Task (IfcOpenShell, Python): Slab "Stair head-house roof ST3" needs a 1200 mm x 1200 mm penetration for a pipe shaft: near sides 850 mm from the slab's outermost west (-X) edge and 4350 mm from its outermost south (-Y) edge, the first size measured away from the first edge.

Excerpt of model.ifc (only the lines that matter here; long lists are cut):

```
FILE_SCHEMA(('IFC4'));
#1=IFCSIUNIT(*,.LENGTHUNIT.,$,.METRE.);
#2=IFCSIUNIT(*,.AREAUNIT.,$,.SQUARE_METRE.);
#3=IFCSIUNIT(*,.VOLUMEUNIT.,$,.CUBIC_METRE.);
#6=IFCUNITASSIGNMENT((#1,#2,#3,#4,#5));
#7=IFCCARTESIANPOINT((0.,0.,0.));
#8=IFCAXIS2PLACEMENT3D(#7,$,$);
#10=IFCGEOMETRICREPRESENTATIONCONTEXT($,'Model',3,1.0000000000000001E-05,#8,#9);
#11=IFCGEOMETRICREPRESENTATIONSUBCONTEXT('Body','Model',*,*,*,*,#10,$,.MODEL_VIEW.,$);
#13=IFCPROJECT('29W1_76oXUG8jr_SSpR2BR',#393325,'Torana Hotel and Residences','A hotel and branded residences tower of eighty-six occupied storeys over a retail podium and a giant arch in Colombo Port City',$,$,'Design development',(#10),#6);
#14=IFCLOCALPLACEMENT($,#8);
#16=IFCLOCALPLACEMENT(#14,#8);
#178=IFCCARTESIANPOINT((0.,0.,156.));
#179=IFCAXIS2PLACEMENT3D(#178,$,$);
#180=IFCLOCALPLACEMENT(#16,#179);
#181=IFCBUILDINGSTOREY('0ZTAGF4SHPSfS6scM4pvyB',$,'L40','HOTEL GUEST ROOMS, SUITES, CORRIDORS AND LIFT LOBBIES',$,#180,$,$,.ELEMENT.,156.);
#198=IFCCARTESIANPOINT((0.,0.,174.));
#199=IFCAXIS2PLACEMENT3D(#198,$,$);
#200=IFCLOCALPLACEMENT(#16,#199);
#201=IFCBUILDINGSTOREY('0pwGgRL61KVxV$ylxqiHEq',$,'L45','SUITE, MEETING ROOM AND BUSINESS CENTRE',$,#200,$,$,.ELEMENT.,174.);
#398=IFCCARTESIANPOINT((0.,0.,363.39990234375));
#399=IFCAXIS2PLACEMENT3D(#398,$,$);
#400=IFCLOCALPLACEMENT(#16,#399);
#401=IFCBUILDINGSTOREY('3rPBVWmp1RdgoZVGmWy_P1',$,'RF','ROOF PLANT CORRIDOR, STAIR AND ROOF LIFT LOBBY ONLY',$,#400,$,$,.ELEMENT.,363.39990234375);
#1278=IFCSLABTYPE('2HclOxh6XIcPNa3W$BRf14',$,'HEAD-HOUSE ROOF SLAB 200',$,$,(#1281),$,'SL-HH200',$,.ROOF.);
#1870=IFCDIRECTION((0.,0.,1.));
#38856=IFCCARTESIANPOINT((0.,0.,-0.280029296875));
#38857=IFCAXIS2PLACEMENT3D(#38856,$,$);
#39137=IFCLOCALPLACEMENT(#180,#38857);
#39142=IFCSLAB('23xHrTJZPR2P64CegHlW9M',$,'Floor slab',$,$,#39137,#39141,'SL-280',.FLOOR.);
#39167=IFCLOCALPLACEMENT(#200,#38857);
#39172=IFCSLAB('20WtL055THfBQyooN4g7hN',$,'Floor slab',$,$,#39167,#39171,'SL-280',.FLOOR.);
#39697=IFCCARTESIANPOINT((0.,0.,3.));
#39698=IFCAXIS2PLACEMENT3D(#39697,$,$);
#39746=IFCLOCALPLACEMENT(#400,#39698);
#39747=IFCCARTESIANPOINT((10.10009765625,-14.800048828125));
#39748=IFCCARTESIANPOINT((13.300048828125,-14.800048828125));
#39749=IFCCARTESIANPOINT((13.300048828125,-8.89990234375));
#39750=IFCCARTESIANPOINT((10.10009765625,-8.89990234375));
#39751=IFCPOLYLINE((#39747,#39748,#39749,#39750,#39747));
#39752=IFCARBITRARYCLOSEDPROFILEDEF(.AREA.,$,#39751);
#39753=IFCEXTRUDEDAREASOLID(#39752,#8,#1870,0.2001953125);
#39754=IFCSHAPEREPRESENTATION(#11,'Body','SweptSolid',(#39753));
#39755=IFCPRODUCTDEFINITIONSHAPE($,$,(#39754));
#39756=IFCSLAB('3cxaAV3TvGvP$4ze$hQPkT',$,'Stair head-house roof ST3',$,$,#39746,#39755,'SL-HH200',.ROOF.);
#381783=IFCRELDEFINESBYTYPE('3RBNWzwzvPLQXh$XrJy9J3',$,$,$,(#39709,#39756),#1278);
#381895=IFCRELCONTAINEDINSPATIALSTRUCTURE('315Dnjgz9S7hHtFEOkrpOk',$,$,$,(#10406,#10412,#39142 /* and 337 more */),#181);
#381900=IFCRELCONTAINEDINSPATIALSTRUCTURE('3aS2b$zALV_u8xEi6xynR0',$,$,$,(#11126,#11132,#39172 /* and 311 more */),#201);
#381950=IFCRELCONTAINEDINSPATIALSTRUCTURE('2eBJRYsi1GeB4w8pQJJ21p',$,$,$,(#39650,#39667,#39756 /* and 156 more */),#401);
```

```python
import numpy as np
import ifcopenshell
import ifcopenshell.api.feature
import ifcopenshell.api.geometry
import ifcopenshell.api.root
import ifcopenshell.geom
import ifcopenshell.util.placement
import ifcopenshell.util.representation
import ifcopenshell.util.shape
import ifcopenshell.util.unit

model = ifcopenshell.open("model.ifc")
unit_scale = ifcopenshell.util.unit.calculate_unit_scale(model)
settings = ifcopenshell.geom.settings()


def volume(element):
    """Net volume in cubic metres, openings subtracted."""
    shape = ifcopenshell.geom.create_shape(settings, element)
    return ifcopenshell.util.shape.get_volume(shape.geometry)


slab = model.by_guid("3cxaAV3TvGvP$4ze$hQPkT")
before = volume(slab)

# Extent in the slab's own axes, in metres. The edges named are its -X and -Y sides.
slab_shape = ifcopenshell.geom.create_shape(settings, slab)
vertices = ifcopenshell.util.shape.get_vertices(slab_shape.geometry)
x_min, y_min, bottom = vertices.min(axis=0)
top = vertices[:, 2].max()

opening = ifcopenshell.api.root.create_entity(model, ifc_class="IfcOpeningElement", name="Pipe shaft opening", predefined_type="OPENING")
context = ifcopenshell.util.representation.get_context(model, "Model", "Body", "MODEL_VIEW")
width, depth = 1.2, 1.2
outline = [(0.0, 0.0), (width, 0.0), (width, depth), (0.0, depth), (0.0, 0.0)]
# Overshoot both faces by 50 mm so the cut is clean.
shape = ifcopenshell.api.geometry.add_slab_representation(
    model, context=context, depth=top - bottom + 0.1, polyline=outline
)
ifcopenshell.api.geometry.assign_representation(model, product=opening, representation=shape)

matrix = ifcopenshell.util.placement.get_local_placement(slab.ObjectPlacement)
matrix[:, 3] = matrix @ np.append(np.array([x_min + 0.85, y_min + 4.35, bottom - 0.05]) / unit_scale, 1.0)
ifcopenshell.api.geometry.edit_object_placement(model, product=opening, matrix=matrix, is_si=False)
ifcopenshell.api.feature.add_feature(model, feature=opening, element=slab)

after = volume(slab)

print(f"slab volume {before:.3f} -> {after:.3f} m3")

model.write("model_rev.ifc")
```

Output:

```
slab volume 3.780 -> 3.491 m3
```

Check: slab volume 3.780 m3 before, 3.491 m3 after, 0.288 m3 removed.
